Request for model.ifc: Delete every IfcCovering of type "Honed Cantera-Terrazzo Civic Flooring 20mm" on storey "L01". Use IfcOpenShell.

First a look at what the model holds.

```python
import ifcopenshell
import ifcopenshell.util.element

model = ifcopenshell.open("model.ifc")
print(model.schema)
storey = next(s for s in model.by_type("IfcBuildingStorey") if s.Name == "L01")
coverings = [e for e in ifcopenshell.util.element.get_decomposition(storey) if e.is_a("IfcCovering")]
seen = {}
for e in coverings:
    element_type = ifcopenshell.util.element.get_type(e)
    name = element_type.Name if element_type not in (None, e) else None
    seen[name] = seen.get(name, 0) + 1
for name, count in sorted(seen.items(), key=str):
    print(count, "x", name)
```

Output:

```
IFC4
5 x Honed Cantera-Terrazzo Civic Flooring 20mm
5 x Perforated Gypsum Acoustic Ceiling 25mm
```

```python
import ifcopenshell
import ifcopenshell.api.root
import ifcopenshell.util.element

model = ifcopenshell.open("model.ifc")

storey = next(s for s in model.by_type("IfcBuildingStorey") if s.Name == "L01")
coverings = [e for e in ifcopenshell.util.element.get_decomposition(storey) if e.is_a("IfcCovering")]
targets = [e for e in coverings if (t := ifcopenshell.util.element.get_type(e)) not in (None, e) and t.Name == "Honed Cantera-Terrazzo Civic Flooring 20mm"]

for e in targets:
    ifcopenshell.api.root.remove_product(model, product=e)
print(len(targets), "removed")

model.write("model_updated.ifc")
```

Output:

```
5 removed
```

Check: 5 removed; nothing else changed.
